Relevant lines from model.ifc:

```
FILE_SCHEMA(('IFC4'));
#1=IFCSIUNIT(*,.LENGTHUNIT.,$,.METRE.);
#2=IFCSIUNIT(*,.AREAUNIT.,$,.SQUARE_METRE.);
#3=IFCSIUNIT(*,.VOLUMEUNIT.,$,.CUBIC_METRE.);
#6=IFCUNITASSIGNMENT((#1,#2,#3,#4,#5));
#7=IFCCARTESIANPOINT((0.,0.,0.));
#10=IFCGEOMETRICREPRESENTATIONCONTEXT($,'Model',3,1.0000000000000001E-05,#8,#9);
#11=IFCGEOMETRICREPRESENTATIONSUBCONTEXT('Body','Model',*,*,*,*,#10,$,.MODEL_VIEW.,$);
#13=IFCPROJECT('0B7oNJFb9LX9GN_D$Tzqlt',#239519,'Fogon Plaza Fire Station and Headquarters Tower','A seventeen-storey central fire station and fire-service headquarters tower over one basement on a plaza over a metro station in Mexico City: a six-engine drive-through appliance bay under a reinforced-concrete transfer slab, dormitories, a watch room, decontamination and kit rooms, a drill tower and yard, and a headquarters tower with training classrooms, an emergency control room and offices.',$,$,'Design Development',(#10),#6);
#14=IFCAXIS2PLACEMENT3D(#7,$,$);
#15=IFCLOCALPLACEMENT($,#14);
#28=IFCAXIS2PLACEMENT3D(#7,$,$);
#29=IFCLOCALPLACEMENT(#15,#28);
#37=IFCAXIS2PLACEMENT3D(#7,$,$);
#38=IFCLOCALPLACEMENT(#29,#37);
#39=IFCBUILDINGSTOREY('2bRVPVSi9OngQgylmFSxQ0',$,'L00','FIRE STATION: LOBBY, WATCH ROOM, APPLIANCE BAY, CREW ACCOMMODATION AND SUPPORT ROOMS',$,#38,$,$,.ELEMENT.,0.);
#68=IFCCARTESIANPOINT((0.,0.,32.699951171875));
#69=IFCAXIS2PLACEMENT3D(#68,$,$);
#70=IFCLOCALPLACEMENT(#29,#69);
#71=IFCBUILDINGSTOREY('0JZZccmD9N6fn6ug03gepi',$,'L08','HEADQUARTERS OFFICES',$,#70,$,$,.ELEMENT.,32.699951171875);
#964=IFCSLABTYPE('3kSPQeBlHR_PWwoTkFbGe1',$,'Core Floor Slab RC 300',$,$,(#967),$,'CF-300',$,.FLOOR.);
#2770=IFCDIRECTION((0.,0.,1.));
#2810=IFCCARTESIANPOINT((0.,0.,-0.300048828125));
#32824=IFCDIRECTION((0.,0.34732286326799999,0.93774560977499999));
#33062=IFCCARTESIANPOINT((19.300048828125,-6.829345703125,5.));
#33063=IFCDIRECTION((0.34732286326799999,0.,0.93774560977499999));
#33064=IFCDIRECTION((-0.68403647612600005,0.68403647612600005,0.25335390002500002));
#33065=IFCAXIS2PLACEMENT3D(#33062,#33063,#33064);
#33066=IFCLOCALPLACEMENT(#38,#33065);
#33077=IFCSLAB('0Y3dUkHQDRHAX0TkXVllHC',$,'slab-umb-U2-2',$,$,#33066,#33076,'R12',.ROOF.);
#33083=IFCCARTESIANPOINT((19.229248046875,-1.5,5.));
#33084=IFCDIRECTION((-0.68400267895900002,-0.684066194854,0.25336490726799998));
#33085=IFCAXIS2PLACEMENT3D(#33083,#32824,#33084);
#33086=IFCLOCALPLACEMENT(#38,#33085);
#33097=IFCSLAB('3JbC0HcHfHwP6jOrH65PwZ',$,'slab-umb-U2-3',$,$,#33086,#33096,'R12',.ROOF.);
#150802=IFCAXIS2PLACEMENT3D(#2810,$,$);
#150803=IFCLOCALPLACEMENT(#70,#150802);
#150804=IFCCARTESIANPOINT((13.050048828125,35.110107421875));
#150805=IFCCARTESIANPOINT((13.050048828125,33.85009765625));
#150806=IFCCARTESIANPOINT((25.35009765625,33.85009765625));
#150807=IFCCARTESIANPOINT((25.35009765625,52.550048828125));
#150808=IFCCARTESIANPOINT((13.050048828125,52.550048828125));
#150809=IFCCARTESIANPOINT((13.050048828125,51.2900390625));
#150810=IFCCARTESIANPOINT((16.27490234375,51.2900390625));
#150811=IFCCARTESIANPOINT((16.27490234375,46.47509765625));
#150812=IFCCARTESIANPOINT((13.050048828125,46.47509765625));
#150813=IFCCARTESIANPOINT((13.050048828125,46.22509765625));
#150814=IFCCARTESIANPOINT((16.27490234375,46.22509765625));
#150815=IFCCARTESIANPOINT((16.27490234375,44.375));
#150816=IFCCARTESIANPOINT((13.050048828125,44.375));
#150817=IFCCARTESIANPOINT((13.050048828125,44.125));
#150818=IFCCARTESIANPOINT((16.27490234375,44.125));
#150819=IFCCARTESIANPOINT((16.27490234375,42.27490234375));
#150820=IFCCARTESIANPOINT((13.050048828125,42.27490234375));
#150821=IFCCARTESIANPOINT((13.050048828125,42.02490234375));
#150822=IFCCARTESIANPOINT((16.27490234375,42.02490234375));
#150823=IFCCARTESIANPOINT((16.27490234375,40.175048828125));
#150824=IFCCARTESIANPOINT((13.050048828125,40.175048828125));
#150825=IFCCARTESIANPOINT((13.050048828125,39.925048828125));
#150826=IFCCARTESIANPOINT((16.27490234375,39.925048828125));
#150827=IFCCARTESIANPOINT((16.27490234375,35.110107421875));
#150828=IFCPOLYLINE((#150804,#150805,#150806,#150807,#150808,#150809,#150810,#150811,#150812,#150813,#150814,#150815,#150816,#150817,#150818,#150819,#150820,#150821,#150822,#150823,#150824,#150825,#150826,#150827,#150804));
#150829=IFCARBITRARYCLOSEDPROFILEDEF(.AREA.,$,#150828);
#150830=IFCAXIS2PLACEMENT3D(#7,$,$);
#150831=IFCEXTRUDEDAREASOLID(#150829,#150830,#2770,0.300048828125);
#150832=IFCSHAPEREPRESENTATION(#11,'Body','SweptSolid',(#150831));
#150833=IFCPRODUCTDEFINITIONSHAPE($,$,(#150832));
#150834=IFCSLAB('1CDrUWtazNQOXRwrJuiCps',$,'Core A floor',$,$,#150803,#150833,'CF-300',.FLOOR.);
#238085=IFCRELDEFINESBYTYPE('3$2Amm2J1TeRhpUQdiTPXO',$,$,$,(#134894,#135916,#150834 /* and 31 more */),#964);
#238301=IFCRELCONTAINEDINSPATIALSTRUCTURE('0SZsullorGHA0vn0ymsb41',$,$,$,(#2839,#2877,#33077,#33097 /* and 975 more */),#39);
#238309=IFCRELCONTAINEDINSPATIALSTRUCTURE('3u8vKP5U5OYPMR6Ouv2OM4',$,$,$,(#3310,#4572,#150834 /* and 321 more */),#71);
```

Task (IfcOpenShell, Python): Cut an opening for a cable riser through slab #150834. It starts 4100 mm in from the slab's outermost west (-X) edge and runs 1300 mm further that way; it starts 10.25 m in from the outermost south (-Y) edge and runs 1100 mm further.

```python
import numpy as np
import ifcopenshell
import ifcopenshell.api.feature
import ifcopenshell.api.geometry
import ifcopenshell.api.root
import ifcopenshell.geom
import ifcopenshell.util.placement
import ifcopenshell.util.representation
import ifcopenshell.util.shape
import ifcopenshell.util.unit

model = ifcopenshell.open("model.ifc")
unit_scale = ifcopenshell.util.unit.calculate_unit_scale(model)
settings = ifcopenshell.geom.settings()


def volume(element):
    """Net volume in cubic metres, openings subtracted."""
    shape = ifcopenshell.geom.create_shape(settings, element)
    return ifcopenshell.util.shape.get_volume(shape.geometry)


slab = model.by_guid("1CDrUWtazNQOXRwrJuiCps")
before = volume(slab)

# Extent in the slab's own axes, in metres. The edges named are its -X and -Y sides.
slab_shape = ifcopenshell.geom.create_shape(settings, slab)
vertices = ifcopenshell.util.shape.get_vertices(slab_shape.geometry)
x_min, y_min, bottom = vertices.min(axis=0)
top = vertices[:, 2].max()

opening = ifcopenshell.api.root.create_entity(model, ifc_class="IfcOpeningElement", name="Cable riser opening", predefined_type="OPENING")
context = ifcopenshell.util.representation.get_context(model, "Model", "Body", "MODEL_VIEW")
width, depth = 1.3, 1.1
outline = [(0.0, 0.0), (width, 0.0), (width, depth), (0.0, depth), (0.0, 0.0)]
# Overshoot both faces by 50 mm so the cut is clean.
shape = ifcopenshell.api.geometry.add_slab_representation(
    model, context=context, depth=top - bottom + 0.1, polyline=outline
)
ifcopenshell.api.geometry.assign_representation(model, product=opening, representation=shape)

matrix = ifcopenshell.util.placement.get_local_placement(slab.ObjectPlacement)
matrix[:, 3] = matrix @ np.append(np.array([x_min + 4.1, y_min + 10.25, bottom - 0.05]) / unit_scale, 1.0)
ifcopenshell.api.geometry.edit_object_placement(model, product=opening, matrix=matrix, is_si=False)
ifcopenshell.api.feature.add_feature(model, feature=opening, element=slab)

after = volume(slab)

print(f"slab volume {before:.3f} -> {after:.3f} m3")

model.write("model_updated.ifc")
```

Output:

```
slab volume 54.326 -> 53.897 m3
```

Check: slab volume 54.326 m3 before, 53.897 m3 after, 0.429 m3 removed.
